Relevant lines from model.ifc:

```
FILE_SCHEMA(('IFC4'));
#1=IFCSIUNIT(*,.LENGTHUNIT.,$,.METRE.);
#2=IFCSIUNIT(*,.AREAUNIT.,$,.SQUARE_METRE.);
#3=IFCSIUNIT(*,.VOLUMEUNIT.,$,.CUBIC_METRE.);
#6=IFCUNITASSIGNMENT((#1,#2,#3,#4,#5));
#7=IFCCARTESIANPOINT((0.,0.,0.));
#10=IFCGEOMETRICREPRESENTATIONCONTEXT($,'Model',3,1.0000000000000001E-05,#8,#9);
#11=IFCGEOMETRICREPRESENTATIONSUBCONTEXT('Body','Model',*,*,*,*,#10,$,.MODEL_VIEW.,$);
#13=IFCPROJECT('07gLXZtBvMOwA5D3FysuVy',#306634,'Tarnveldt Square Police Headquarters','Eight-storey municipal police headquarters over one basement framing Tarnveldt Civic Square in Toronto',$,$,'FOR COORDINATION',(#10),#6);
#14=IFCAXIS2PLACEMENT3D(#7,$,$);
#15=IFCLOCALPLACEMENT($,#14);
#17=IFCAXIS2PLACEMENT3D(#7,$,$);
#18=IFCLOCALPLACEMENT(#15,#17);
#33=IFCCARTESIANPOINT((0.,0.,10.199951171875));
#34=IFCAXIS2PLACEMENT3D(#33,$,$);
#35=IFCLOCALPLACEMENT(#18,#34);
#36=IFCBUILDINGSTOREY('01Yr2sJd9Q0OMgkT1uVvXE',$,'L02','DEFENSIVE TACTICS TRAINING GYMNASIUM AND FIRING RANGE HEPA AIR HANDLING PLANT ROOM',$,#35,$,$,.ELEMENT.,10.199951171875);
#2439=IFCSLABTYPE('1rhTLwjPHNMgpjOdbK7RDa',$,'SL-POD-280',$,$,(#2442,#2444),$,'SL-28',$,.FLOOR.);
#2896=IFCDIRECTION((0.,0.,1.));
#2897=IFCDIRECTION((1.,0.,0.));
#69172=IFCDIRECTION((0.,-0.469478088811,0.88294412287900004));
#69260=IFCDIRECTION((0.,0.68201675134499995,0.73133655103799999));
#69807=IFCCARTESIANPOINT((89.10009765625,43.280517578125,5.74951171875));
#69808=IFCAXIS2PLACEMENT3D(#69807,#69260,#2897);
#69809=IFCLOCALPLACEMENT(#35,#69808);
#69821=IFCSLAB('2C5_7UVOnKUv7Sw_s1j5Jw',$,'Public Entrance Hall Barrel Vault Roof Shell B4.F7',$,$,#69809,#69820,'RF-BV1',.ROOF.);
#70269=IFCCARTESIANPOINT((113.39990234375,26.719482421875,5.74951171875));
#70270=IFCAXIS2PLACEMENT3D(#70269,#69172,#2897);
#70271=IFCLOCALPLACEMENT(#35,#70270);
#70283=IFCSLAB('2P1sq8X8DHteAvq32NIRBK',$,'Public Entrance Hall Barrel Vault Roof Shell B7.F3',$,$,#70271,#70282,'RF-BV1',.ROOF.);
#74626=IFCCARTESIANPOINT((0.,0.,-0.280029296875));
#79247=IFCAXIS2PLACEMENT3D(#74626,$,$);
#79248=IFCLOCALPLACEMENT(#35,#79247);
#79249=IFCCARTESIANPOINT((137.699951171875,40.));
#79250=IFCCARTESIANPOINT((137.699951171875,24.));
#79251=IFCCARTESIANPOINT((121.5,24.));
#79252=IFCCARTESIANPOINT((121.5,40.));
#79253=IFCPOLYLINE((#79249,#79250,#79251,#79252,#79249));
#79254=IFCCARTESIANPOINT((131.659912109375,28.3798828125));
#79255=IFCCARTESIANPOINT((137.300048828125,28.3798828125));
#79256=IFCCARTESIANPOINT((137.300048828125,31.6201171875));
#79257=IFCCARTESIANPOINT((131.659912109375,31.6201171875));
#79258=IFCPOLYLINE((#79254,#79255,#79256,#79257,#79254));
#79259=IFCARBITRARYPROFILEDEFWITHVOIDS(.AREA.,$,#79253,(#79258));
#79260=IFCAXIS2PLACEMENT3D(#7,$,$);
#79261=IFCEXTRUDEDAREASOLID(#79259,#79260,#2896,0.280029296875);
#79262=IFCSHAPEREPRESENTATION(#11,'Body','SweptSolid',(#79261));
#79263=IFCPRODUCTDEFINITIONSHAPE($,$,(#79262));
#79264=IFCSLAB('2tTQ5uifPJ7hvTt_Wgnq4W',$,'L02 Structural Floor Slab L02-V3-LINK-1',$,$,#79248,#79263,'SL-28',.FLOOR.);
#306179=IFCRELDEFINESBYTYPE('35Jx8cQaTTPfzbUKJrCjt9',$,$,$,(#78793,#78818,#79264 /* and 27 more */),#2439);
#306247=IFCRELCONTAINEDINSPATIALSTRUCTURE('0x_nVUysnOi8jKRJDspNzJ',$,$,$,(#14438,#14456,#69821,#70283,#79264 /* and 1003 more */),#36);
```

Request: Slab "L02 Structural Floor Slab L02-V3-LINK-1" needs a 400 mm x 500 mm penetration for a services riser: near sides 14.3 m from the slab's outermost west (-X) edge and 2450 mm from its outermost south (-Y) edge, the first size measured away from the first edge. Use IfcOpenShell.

```python
import numpy as np
import ifcopenshell
import ifcopenshell.api.feature
import ifcopenshell.api.geometry
import ifcopenshell.api.root
import ifcopenshell.geom
import ifcopenshell.util.placement
import ifcopenshell.util.representation
import ifcopenshell.util.shape
import ifcopenshell.util.unit

model = ifcopenshell.open("model.ifc")
unit_scale = ifcopenshell.util.unit.calculate_unit_scale(model)
settings = ifcopenshell.geom.settings()


def volume(element):
    """Net volume in cubic metres, openings subtracted."""
    shape = ifcopenshell.geom.create_shape(settings, element)
    return ifcopenshell.util.shape.get_volume(shape.geometry)


slab = model.by_id(79264)
before = volume(slab)

# Extent in the slab's own axes, in metres. The edges named are its -X and -Y sides.
slab_shape = ifcopenshell.geom.create_shape(settings, slab)
vertices = ifcopenshell.util.shape.get_vertices(slab_shape.geometry)
x_min, y_min, bottom = vertices.min(axis=0)
top = vertices[:, 2].max()

opening = ifcopenshell.api.root.create_entity(model, ifc_class="IfcOpeningElement", name="Services riser opening", predefined_type="OPENING")
context = ifcopenshell.util.representation.get_context(model, "Model", "Body", "MODEL_VIEW")
width, depth = 0.4, 0.5
outline = [(0.0, 0.0), (width, 0.0), (width, depth), (0.0, depth), (0.0, 0.0)]
# Overshoot both faces by 50 mm so the cut is clean.
shape = ifcopenshell.api.geometry.add_slab_representation(
    model, context=context, depth=top - bottom + 0.1, polyline=outline
)
ifcopenshell.api.geometry.assign_representation(model, product=opening, representation=shape)

matrix = ifcopenshell.util.placement.get_local_placement(slab.ObjectPlacement)
matrix[:, 3] = matrix @ np.append(np.array([x_min + 14.3, y_min + 2.45, bottom - 0.05]) / unit_scale, 1.0)
ifcopenshell.api.geometry.edit_object_placement(model, product=opening, matrix=matrix, is_si=False)
ifcopenshell.api.feature.add_feature(model, feature=opening, element=slab)

after = volume(slab)

print(f"slab volume {before:.3f} -> {after:.3f} m3")

model.write("model-out.ifc")
```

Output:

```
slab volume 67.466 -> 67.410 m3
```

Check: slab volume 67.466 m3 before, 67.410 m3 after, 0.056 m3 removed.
